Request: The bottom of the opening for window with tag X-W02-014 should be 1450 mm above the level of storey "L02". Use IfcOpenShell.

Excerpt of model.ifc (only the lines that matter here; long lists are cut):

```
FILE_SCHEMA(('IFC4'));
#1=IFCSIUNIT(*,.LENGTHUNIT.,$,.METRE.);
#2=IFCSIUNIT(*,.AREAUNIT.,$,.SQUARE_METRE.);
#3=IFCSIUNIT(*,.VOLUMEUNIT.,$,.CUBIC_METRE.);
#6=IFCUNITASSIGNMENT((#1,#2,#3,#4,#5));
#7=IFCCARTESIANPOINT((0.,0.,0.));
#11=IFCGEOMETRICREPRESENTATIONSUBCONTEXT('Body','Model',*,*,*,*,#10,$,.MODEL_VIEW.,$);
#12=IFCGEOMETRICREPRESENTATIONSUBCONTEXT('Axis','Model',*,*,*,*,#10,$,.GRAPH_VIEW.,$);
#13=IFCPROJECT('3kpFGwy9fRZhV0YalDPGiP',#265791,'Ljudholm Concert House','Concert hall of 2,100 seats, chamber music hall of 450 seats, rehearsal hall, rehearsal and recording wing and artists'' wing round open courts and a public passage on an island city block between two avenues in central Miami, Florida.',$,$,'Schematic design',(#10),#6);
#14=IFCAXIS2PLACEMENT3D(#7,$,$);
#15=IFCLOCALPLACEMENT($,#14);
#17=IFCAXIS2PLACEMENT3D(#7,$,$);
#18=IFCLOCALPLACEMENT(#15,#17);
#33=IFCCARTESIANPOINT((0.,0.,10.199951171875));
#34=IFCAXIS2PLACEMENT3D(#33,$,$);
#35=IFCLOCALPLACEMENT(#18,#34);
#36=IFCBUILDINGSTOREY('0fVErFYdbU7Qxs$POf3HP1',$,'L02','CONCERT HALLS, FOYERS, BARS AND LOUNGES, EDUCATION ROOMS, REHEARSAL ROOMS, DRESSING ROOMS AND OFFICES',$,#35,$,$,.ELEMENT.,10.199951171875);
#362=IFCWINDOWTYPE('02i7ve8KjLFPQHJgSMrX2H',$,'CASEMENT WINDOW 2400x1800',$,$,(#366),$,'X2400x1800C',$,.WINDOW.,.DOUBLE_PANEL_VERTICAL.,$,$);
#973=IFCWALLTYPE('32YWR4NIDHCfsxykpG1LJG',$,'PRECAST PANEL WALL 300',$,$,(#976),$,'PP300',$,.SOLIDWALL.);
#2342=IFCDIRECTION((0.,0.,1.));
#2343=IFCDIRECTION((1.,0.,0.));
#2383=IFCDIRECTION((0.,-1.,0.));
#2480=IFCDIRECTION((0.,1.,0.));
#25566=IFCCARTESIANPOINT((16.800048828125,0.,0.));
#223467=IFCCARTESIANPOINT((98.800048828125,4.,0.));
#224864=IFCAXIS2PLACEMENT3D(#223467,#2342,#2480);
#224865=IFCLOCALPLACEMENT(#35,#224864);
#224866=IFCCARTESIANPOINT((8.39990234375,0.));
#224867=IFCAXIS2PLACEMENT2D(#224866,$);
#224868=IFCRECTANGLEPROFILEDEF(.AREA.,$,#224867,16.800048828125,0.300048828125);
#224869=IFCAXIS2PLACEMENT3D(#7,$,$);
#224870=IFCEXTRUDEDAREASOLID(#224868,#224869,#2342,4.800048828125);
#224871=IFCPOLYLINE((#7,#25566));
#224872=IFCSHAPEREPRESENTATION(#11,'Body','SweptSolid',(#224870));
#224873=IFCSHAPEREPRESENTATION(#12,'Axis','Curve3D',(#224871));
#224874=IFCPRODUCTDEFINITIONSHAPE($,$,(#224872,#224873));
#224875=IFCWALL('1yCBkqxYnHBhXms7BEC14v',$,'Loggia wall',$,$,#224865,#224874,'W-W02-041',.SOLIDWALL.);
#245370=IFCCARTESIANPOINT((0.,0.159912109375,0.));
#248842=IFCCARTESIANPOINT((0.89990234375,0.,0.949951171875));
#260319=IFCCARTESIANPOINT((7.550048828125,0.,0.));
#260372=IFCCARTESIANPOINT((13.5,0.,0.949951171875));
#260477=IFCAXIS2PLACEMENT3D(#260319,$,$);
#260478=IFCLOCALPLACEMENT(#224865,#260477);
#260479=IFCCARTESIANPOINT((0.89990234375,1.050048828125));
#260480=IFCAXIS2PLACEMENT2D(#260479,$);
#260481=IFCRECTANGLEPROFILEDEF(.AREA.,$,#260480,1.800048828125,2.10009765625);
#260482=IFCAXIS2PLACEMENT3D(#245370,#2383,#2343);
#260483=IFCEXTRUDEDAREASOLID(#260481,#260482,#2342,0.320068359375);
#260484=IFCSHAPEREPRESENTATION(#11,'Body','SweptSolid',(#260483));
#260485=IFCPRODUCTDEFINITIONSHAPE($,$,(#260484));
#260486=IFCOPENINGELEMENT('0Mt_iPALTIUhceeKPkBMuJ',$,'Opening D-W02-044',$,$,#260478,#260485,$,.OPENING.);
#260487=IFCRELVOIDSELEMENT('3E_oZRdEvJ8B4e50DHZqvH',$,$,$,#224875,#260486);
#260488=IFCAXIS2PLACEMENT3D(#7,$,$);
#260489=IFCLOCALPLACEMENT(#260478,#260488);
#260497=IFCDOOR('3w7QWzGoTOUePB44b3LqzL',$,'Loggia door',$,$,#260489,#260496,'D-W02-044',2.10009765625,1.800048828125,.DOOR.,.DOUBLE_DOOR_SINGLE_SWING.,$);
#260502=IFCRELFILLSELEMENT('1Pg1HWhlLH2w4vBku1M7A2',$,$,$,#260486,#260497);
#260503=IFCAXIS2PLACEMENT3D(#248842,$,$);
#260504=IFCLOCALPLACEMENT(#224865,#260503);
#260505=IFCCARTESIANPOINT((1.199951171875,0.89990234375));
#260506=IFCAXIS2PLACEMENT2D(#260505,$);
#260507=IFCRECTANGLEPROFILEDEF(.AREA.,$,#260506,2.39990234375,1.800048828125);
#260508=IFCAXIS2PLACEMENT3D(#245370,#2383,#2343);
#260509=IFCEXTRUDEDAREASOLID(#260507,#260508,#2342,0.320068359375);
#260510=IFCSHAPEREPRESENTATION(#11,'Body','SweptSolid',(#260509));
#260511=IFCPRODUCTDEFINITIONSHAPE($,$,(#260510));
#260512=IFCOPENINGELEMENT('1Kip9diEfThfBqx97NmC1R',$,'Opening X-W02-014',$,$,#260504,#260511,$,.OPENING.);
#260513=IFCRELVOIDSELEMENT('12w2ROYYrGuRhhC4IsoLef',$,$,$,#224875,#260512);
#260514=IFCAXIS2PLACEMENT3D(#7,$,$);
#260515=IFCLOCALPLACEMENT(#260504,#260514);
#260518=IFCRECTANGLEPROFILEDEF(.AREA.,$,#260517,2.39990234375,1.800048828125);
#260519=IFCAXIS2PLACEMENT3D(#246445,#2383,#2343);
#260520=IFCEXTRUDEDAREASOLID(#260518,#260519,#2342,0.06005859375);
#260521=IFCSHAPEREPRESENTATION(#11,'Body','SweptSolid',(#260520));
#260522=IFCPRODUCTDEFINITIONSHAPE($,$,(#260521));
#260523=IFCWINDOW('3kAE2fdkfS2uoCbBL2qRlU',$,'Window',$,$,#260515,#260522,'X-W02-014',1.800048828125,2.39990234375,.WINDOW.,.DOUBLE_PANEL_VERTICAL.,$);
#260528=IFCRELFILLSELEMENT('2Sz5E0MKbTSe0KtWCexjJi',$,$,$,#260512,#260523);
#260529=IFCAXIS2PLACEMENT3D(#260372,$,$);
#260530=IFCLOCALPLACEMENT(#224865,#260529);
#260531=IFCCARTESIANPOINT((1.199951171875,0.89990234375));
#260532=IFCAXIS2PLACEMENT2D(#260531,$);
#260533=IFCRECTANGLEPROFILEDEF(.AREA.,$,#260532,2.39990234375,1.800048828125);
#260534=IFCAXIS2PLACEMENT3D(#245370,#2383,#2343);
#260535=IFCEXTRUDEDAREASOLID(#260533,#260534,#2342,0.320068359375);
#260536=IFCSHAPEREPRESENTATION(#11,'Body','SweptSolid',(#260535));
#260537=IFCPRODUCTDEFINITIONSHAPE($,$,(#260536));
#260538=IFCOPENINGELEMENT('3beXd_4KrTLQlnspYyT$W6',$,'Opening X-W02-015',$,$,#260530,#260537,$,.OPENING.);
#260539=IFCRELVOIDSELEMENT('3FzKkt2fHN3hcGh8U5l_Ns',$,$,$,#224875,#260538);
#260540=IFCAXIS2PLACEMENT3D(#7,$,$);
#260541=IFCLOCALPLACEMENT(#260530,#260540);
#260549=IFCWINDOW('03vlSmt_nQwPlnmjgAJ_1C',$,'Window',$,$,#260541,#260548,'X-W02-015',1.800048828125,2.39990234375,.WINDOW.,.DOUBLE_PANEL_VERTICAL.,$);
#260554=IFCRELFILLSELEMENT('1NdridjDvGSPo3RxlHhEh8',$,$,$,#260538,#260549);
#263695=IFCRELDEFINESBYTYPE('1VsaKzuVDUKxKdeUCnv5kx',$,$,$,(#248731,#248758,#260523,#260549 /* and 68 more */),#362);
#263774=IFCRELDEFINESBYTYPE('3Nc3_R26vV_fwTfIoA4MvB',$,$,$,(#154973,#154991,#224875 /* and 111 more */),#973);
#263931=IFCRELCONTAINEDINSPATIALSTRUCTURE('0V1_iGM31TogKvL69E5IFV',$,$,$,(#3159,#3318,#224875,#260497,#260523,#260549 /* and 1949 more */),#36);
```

```python
import numpy as np
import ifcopenshell
import ifcopenshell.api.geometry
import ifcopenshell.geom
import ifcopenshell.util.element
import ifcopenshell.util.placement
import ifcopenshell.util.shape
import ifcopenshell.util.unit

model = ifcopenshell.open("model.ifc")
unit_scale = ifcopenshell.util.unit.calculate_unit_scale(model)

window = model.by_id(260523)
opening = window.FillsVoids[0].RelatingOpeningElement
storey = ifcopenshell.util.element.get_container(window, ifc_class="IfcBuildingStorey")
level = ifcopenshell.util.placement.get_local_placement(storey.ObjectPlacement)[2, 3]

# The opening's origin need not be at the sill, so measure its lowest point.
shape = ifcopenshell.geom.create_shape(ifcopenshell.geom.settings(), opening)
bottom = ifcopenshell.util.shape.get_shape_bottom_elevation(shape, shape.geometry) / unit_scale
dz = level + 1.45 / unit_scale - bottom

shift = np.array([0.0, 0.0, dz])
# The window is placed relative to its opening, so it follows when the opening moves.
matrix = ifcopenshell.util.placement.get_local_placement(opening.ObjectPlacement)
matrix[:3, 3] += shift
ifcopenshell.api.geometry.edit_object_placement(
    model, product=opening, matrix=matrix, is_si=False, should_transform_children=True
)

print(f"moved by {dz * unit_scale:+.3f} m")

model.write("model_updated.ifc")
```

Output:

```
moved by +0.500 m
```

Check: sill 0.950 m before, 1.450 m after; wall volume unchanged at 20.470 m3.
